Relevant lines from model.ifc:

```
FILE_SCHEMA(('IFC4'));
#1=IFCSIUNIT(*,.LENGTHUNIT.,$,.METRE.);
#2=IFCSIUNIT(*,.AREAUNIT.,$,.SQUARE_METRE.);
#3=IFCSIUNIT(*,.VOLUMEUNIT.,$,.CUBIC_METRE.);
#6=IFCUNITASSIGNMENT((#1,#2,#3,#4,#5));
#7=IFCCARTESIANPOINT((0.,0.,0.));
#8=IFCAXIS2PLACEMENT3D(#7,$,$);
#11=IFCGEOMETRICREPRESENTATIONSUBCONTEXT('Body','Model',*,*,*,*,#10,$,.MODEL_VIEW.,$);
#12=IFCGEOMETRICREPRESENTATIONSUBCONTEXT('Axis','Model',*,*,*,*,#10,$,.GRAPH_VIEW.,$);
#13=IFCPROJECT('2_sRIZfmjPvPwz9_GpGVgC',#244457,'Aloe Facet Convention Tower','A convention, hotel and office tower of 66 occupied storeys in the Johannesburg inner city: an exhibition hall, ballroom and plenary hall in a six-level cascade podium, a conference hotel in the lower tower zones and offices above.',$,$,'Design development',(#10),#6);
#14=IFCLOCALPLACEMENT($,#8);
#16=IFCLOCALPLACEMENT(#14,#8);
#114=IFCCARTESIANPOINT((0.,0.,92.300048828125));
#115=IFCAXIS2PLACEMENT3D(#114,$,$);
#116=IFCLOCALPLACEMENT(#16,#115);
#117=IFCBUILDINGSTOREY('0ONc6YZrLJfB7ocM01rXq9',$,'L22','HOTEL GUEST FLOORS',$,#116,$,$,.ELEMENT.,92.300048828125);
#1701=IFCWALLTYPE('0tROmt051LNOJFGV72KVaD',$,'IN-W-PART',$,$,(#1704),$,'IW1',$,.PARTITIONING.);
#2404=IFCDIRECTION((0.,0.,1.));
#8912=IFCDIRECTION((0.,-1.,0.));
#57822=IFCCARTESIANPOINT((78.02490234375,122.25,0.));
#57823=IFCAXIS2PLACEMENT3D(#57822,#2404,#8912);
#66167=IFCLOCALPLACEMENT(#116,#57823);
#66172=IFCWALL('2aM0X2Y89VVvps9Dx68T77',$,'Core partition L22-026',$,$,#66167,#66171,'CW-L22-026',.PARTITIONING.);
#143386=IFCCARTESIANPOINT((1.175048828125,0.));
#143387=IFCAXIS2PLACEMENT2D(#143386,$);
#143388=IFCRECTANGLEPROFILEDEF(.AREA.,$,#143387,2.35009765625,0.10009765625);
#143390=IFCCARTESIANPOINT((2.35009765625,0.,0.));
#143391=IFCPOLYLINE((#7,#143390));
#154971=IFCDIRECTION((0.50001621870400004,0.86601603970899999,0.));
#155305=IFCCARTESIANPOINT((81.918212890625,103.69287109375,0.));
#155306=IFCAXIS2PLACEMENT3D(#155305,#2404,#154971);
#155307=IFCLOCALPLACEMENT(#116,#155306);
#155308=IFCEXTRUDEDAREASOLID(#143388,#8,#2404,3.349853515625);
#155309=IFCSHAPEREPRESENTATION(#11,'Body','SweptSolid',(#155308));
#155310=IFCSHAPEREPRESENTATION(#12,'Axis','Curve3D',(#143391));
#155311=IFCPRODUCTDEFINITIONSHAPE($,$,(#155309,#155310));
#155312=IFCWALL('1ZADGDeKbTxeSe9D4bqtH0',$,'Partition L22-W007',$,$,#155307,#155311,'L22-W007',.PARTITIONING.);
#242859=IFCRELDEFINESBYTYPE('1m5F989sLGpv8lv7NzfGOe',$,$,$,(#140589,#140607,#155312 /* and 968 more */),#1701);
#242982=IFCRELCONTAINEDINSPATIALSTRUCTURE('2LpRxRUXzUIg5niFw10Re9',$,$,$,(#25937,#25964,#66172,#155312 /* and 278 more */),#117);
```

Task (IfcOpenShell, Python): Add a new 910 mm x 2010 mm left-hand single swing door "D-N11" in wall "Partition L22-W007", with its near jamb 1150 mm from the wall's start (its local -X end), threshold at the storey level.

```python
import numpy as np
import ifcopenshell
import ifcopenshell.api.feature
import ifcopenshell.api.geometry
import ifcopenshell.api.root
import ifcopenshell.api.spatial
import ifcopenshell.geom
import ifcopenshell.util.element
import ifcopenshell.util.placement
import ifcopenshell.util.representation
import ifcopenshell.util.shape
import ifcopenshell.util.unit

model = ifcopenshell.open("model.ifc")
unit_scale = ifcopenshell.util.unit.calculate_unit_scale(model)
settings = ifcopenshell.geom.settings()


def volume(element):
    """Net volume in cubic metres, openings subtracted."""
    shape = ifcopenshell.geom.create_shape(settings, element)
    return ifcopenshell.util.shape.get_volume(shape.geometry)


wall = model.by_guid("1ZADGDeKbTxeSe9D4bqtH0")
storey = ifcopenshell.util.element.get_container(wall, ifc_class="IfcBuildingStorey")
context = ifcopenshell.util.representation.get_context(model, "Model", "Body", "MODEL_VIEW")
before = volume(wall)

width, height, from_end, sill = 0.91, 2.01, 1.15, 0.0  # metres

# The wall runs along its own X axis, and the end named is its -X end.
wall_shape = ifcopenshell.geom.create_shape(settings, wall)
x, y, z = ifcopenshell.util.shape.get_vertices(wall_shape.geometry).T
start = x.min() + from_end
face, thickness = float(y.min()), float(y.max() - y.min())
wall_matrix = ifcopenshell.util.placement.get_local_placement(wall.ObjectPlacement)
level = ifcopenshell.util.placement.get_local_placement(storey.ObjectPlacement)[2, 3]


def in_wall(x, y):
    """Placement at x, y metres in the wall's axes, at sill height."""
    matrix = wall_matrix.copy()
    matrix[:, 3] = wall_matrix @ np.array([x / unit_scale, y / unit_scale, 0.0, 1.0])
    matrix[2, 3] = level + sill / unit_scale
    return matrix


# Opening: a box that overshoots both wall faces by 50 mm.
opening = ifcopenshell.api.root.create_entity(model, ifc_class="IfcOpeningElement", predefined_type="OPENING")
box = ifcopenshell.api.geometry.add_wall_representation(
    model, context=context, length=width, height=height, thickness=thickness + 0.1
)
ifcopenshell.api.geometry.assign_representation(model, product=opening, representation=box)
ifcopenshell.api.geometry.edit_object_placement(model, product=opening, matrix=in_wall(start, face - 0.05), is_si=False)
ifcopenshell.api.feature.add_feature(model, feature=opening, element=wall)

door = ifcopenshell.api.root.create_entity(model, ifc_class="IfcDoor", name="D-N11", predefined_type="DOOR")
door.OverallWidth, door.OverallHeight = width / unit_scale, height / unit_scale
door.OperationType = "SINGLE_SWING_LEFT"
body = ifcopenshell.api.geometry.add_door_representation(
    model,
    context=context,
    overall_width=door.OverallWidth,
    overall_height=door.OverallHeight,
    operation_type="SINGLE_SWING_LEFT",
    lining_properties={"LiningDepth": thickness / unit_scale, "ThresholdDepth": thickness / unit_scale},
)
ifcopenshell.api.geometry.assign_representation(model, product=door, representation=body)
ifcopenshell.api.spatial.assign_container(model, products=[door], relating_structure=storey)
ifcopenshell.api.feature.add_filling(model, opening=opening, element=door)

# The lining spans the wall, so the door starts at the wall face.
ifcopenshell.api.geometry.edit_object_placement(model, product=door, matrix=in_wall(start, face), is_si=False)

after = volume(wall)

print(f"wall volume {before:.3f} -> {after:.3f} m3")

model.write("model_updated.ifc")
```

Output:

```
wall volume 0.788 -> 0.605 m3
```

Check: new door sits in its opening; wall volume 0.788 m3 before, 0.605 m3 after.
